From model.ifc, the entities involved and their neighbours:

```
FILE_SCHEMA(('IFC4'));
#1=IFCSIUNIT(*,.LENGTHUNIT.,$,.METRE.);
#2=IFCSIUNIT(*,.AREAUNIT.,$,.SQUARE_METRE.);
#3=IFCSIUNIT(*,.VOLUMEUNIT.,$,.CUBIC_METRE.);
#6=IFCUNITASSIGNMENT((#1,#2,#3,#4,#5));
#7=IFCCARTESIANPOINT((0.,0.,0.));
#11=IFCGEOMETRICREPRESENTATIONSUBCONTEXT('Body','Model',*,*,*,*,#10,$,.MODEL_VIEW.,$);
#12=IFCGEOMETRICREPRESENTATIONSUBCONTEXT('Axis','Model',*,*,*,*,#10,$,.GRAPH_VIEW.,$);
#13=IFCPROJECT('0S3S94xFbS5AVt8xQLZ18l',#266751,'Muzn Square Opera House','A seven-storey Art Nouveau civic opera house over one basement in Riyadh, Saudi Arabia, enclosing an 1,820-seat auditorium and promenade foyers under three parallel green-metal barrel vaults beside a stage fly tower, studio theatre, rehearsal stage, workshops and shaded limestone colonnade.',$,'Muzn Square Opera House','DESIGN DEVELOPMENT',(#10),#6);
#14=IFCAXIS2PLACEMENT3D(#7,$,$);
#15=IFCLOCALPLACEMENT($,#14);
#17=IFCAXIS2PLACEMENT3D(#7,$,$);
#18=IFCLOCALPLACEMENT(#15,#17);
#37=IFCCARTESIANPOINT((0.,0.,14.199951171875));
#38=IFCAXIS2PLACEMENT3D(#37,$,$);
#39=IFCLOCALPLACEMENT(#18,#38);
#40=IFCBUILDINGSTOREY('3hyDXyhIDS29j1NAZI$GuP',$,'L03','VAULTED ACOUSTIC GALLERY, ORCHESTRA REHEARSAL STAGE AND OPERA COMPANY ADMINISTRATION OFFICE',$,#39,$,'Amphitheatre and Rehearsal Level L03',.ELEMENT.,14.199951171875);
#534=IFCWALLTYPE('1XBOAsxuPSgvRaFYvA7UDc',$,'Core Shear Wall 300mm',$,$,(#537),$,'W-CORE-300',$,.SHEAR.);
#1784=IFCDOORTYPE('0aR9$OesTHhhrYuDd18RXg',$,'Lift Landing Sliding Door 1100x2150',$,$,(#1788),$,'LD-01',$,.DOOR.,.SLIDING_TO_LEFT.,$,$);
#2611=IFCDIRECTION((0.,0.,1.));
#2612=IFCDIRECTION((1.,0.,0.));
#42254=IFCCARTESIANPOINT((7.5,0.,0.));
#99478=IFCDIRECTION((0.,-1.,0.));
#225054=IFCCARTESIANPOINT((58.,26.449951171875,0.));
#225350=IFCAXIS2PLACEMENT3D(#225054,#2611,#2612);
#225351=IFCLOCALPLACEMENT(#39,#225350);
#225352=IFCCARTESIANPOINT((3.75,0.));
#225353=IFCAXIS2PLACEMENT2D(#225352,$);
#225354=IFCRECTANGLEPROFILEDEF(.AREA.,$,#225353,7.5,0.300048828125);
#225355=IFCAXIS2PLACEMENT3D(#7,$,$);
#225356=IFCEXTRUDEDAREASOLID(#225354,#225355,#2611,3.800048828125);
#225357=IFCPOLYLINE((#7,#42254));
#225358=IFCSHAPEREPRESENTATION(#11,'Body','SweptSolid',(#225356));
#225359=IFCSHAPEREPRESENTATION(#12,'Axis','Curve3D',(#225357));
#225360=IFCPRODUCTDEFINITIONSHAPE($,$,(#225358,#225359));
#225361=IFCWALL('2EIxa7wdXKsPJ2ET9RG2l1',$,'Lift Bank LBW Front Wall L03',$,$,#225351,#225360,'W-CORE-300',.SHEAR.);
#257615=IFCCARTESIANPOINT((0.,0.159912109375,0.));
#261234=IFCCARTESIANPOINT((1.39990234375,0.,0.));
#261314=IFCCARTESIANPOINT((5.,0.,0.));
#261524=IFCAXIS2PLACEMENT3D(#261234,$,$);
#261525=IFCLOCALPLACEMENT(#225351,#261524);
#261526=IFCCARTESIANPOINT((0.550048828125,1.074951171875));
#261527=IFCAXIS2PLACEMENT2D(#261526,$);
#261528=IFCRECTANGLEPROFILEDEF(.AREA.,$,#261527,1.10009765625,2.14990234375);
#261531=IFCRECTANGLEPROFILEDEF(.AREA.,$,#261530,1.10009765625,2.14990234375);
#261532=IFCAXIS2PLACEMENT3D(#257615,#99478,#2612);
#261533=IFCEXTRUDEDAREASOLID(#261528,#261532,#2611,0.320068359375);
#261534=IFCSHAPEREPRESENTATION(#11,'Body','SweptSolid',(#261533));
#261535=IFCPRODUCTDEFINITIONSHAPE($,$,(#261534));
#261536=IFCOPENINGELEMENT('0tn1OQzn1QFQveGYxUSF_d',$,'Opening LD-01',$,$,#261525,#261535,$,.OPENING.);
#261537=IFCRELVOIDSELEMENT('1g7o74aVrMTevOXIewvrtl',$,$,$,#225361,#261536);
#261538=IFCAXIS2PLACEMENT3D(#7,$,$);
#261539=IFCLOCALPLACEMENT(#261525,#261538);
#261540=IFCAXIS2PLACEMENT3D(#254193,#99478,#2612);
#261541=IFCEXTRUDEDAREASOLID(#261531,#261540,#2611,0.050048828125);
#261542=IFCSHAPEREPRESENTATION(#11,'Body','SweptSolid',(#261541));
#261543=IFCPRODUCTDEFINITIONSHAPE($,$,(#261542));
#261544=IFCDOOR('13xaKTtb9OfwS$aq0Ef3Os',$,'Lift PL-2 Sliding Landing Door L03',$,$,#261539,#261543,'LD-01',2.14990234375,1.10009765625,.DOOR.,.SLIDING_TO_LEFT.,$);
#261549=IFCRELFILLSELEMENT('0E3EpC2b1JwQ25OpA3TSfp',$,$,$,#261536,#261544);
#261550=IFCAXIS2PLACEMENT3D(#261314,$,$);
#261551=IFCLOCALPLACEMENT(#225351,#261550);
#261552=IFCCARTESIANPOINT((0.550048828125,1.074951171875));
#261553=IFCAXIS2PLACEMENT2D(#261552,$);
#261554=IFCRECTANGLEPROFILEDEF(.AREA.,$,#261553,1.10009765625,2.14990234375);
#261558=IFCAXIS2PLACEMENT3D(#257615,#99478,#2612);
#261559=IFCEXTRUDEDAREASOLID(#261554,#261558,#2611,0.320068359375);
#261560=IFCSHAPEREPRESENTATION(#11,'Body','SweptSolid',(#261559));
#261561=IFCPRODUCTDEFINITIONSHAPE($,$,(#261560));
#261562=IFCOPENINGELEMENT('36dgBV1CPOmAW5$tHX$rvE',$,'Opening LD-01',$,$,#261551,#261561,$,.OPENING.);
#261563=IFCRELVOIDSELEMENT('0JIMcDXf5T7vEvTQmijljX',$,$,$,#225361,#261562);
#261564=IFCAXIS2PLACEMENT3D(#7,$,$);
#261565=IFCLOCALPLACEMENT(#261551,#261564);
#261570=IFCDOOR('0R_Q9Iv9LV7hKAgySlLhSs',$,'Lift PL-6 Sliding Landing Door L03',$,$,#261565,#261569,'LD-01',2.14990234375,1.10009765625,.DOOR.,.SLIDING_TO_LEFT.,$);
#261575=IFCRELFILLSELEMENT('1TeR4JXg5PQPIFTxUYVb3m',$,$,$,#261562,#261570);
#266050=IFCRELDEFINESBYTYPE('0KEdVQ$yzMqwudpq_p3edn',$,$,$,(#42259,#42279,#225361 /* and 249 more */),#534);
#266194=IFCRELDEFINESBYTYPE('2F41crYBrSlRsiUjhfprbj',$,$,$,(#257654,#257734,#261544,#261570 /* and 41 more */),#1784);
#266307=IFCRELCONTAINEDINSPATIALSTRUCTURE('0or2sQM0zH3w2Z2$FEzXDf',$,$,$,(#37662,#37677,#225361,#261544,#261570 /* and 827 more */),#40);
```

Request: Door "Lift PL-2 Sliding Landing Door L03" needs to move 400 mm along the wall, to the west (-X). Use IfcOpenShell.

```python
import ifcopenshell
import ifcopenshell.api.geometry
import ifcopenshell.util.placement
import ifcopenshell.util.unit

model = ifcopenshell.open("model.ifc")
unit_scale = ifcopenshell.util.unit.calculate_unit_scale(model)

door = model.by_guid("13xaKTtb9OfwS$aq0Ef3Os")
opening = door.FillsVoids[0].RelatingOpeningElement
wall = opening.VoidsElements[0].RelatingBuildingElement

wall_matrix = ifcopenshell.util.placement.get_local_placement(wall.ObjectPlacement)
shift = wall_matrix[:3, 0] * -0.4 / unit_scale
before = ifcopenshell.util.placement.get_local_placement(door.ObjectPlacement)[:3, 3].copy()

# The door is placed relative to its opening, so it follows when the opening moves.
matrix = ifcopenshell.util.placement.get_local_placement(opening.ObjectPlacement)
matrix[:3, 3] += shift
ifcopenshell.api.geometry.edit_object_placement(
    model, product=opening, matrix=matrix, is_si=False, should_transform_children=True
)

after = ifcopenshell.util.placement.get_local_placement(door.ObjectPlacement)[:3, 3]
print("door moved by", (after - before).round(3) + 0.0)

model.write("model_v2.ifc")
```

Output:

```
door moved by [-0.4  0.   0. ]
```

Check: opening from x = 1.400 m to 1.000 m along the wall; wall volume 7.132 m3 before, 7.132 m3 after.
